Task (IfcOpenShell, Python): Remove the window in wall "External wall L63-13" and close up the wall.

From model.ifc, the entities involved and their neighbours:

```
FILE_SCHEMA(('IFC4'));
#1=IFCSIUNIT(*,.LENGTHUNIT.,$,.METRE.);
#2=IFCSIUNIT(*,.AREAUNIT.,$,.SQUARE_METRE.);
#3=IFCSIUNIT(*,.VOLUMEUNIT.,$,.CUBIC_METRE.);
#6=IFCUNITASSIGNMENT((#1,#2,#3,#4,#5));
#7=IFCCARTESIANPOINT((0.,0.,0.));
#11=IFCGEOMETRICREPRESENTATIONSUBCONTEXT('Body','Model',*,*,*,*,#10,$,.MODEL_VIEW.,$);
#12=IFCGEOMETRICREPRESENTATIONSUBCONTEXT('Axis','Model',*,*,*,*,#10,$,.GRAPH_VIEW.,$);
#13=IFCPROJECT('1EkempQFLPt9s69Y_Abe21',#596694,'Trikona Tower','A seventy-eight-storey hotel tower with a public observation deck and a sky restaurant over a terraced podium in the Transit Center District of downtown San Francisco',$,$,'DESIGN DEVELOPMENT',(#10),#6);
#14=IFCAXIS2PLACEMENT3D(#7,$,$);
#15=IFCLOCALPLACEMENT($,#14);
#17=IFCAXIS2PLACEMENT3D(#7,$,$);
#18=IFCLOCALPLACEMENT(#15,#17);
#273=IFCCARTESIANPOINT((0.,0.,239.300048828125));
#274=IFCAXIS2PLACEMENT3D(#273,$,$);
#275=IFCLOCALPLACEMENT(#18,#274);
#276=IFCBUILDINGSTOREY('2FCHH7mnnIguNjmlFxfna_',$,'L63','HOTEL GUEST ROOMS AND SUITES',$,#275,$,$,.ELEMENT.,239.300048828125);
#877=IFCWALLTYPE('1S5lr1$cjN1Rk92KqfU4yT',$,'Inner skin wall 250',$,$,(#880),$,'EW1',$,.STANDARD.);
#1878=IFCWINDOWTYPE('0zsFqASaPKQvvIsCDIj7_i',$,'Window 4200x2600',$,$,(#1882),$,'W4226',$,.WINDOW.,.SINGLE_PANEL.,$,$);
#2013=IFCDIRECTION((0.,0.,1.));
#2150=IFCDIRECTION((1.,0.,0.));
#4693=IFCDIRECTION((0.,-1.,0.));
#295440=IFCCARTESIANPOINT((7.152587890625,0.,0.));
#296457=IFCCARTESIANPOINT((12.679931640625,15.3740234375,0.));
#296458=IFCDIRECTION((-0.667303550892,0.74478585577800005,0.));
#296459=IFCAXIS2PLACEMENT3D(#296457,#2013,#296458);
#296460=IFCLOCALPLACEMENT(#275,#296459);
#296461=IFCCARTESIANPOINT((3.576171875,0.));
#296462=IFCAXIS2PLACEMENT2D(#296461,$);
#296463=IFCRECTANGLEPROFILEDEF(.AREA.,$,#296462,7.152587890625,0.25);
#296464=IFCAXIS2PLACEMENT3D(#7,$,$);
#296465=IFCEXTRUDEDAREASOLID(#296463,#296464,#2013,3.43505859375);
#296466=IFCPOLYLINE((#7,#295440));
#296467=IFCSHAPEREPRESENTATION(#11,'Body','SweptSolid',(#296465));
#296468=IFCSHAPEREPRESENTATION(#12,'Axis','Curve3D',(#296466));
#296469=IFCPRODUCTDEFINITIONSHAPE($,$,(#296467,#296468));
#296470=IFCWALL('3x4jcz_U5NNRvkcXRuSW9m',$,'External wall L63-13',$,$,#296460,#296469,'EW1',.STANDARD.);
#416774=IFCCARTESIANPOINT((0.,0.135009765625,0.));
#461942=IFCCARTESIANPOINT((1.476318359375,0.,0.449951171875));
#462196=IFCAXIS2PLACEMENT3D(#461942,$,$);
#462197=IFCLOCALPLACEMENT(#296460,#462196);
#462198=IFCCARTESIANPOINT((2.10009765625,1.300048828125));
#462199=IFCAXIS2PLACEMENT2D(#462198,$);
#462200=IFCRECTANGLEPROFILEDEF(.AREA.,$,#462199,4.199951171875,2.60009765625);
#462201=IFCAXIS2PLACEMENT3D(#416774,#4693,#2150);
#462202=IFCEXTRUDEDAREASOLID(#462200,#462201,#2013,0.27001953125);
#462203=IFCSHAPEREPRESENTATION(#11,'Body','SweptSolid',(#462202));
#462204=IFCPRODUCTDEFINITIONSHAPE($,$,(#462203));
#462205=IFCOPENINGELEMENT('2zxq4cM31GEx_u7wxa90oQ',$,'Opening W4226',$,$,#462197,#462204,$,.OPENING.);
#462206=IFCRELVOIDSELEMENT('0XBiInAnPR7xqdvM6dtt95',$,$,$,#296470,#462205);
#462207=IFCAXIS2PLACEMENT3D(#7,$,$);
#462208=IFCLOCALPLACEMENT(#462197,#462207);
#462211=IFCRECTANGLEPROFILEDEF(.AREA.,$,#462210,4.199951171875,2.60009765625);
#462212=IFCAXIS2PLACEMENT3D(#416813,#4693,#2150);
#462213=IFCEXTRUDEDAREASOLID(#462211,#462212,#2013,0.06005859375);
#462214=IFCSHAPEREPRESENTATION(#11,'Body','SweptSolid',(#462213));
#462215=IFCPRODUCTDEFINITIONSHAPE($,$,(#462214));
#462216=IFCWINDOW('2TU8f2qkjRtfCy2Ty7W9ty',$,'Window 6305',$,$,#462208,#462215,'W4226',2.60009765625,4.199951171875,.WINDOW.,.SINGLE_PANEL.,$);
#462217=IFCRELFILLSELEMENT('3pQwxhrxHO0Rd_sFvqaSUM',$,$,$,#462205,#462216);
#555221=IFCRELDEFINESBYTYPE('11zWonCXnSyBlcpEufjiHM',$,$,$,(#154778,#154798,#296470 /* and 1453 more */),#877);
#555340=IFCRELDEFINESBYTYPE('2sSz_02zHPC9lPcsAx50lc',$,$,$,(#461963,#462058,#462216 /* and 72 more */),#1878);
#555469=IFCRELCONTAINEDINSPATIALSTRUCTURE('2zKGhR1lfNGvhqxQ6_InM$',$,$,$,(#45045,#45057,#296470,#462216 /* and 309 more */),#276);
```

```python
import ifcopenshell
import ifcopenshell.api.feature
import ifcopenshell.api.root
import ifcopenshell.geom
import ifcopenshell.util.shape

model = ifcopenshell.open("model.ifc")
settings = ifcopenshell.geom.settings()


def volume(element):
    """Net volume in cubic metres, openings subtracted."""
    shape = ifcopenshell.geom.create_shape(settings, element)
    return ifcopenshell.util.shape.get_volume(shape.geometry)


window = model.by_id(462216)
opening = window.FillsVoids[0].RelatingOpeningElement
wall = opening.VoidsElements[0].RelatingBuildingElement
before = volume(wall)

ifcopenshell.api.root.remove_product(model, product=window)
ifcopenshell.api.feature.remove_feature(model, feature=opening)

after = volume(wall)

print(f"wall volume {before:.3f} -> {after:.3f} m3")

model.write("model_updated.ifc")
```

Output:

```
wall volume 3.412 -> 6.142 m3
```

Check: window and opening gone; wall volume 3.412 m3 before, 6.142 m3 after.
